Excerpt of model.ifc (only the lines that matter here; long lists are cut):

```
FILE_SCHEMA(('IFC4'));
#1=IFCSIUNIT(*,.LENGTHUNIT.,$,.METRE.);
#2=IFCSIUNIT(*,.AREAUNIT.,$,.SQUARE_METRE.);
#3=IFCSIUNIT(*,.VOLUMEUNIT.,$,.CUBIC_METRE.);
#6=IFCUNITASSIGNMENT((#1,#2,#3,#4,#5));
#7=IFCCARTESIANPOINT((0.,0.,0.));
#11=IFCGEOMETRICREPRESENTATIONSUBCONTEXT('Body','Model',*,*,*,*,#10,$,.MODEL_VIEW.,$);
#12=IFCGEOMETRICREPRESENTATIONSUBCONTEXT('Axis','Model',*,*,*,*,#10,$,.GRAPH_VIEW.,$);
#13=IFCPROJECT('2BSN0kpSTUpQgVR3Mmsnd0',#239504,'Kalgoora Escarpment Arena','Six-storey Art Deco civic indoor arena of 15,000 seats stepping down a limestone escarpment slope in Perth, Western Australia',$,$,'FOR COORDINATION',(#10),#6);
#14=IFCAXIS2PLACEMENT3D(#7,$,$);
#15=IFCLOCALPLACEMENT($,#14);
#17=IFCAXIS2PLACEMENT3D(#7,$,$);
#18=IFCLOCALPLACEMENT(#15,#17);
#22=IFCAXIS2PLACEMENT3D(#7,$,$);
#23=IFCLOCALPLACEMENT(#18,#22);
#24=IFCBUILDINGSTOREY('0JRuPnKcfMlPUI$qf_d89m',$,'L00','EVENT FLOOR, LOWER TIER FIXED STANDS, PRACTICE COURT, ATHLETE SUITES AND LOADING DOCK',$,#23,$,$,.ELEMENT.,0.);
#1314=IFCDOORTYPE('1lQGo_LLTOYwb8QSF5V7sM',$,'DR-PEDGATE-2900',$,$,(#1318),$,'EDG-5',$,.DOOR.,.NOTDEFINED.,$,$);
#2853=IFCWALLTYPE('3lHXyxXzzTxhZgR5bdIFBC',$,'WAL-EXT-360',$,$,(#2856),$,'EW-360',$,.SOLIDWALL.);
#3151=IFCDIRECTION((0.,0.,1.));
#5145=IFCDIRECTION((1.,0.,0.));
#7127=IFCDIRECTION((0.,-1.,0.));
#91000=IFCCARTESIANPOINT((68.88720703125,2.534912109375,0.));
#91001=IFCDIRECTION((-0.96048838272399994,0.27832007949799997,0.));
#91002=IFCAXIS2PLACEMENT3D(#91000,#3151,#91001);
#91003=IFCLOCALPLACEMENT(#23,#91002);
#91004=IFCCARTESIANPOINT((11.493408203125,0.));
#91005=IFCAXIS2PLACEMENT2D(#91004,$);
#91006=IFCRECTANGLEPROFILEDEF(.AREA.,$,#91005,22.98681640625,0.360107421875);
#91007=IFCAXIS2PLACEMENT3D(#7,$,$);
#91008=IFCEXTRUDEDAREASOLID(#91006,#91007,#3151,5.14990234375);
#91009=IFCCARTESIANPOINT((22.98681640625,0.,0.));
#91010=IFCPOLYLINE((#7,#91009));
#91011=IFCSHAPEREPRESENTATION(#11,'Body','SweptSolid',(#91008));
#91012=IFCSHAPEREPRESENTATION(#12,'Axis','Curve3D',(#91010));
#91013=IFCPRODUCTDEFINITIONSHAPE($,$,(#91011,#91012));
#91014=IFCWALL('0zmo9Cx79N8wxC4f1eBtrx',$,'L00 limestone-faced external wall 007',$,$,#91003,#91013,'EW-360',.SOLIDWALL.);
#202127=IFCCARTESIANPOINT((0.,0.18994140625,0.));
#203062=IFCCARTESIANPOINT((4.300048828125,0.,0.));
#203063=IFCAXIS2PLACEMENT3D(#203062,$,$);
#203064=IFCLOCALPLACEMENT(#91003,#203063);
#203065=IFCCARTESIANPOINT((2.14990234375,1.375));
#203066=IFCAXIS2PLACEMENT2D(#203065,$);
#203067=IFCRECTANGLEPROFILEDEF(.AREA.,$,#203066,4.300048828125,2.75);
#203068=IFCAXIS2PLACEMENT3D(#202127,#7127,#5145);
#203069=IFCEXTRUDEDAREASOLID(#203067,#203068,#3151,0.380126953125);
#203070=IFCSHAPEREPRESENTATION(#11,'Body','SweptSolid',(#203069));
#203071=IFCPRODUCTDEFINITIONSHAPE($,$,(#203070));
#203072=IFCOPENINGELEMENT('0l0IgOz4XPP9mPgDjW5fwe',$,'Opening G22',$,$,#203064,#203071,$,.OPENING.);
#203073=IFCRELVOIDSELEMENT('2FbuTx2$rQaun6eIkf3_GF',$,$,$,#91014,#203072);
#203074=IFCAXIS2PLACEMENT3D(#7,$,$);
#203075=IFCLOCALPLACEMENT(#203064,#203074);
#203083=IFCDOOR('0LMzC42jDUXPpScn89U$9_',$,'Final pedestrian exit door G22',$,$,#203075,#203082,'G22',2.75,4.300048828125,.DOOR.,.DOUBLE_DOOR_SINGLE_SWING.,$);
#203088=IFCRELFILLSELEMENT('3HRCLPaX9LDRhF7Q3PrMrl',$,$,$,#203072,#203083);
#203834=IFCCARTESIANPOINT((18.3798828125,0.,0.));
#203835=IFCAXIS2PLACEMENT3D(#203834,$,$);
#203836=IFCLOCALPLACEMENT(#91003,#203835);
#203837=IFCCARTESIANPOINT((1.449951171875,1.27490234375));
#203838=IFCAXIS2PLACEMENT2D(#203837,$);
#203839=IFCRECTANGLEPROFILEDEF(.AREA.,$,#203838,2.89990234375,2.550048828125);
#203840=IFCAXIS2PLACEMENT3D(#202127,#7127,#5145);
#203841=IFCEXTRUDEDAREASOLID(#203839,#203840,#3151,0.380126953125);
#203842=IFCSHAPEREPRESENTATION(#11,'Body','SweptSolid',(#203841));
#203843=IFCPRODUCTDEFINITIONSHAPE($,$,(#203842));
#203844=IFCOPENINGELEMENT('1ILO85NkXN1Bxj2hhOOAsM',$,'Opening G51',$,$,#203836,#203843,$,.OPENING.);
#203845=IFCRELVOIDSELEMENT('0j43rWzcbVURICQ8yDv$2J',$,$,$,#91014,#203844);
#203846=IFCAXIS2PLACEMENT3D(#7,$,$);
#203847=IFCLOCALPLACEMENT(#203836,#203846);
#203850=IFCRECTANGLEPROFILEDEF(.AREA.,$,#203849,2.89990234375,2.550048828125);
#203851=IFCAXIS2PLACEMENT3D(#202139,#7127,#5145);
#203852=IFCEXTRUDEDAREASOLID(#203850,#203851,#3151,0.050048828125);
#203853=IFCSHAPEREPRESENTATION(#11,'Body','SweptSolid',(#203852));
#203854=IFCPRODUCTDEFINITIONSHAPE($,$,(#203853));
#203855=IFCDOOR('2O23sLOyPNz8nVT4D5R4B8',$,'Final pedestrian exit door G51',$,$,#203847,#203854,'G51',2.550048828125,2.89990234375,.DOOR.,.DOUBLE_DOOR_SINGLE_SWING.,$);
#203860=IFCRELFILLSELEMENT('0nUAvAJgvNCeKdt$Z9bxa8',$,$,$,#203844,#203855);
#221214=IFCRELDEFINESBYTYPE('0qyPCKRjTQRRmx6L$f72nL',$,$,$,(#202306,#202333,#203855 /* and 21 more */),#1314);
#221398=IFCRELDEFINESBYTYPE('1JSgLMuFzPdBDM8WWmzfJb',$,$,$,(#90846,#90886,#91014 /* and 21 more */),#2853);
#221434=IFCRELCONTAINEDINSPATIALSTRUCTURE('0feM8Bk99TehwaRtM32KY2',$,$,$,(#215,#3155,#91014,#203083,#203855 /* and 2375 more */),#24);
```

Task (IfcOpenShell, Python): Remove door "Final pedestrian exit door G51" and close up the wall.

```python
import ifcopenshell
import ifcopenshell.api.feature
import ifcopenshell.api.root
import ifcopenshell.geom
import ifcopenshell.util.shape

model = ifcopenshell.open("model.ifc")
settings = ifcopenshell.geom.settings()


def volume(element):
    """Net volume in cubic metres, openings subtracted."""
    shape = ifcopenshell.geom.create_shape(settings, element)
    return ifcopenshell.util.shape.get_volume(shape.geometry)


door = model.by_id(203855)
opening = door.FillsVoids[0].RelatingOpeningElement
wall = opening.VoidsElements[0].RelatingBuildingElement
before = volume(wall)

ifcopenshell.api.root.remove_product(model, product=door)
ifcopenshell.api.feature.remove_feature(model, feature=opening)

after = volume(wall)

print(f"wall volume {before:.3f} -> {after:.3f} m3")

model.write("model-out.ifc")
```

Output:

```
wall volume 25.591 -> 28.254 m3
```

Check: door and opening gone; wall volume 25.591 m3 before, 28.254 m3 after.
